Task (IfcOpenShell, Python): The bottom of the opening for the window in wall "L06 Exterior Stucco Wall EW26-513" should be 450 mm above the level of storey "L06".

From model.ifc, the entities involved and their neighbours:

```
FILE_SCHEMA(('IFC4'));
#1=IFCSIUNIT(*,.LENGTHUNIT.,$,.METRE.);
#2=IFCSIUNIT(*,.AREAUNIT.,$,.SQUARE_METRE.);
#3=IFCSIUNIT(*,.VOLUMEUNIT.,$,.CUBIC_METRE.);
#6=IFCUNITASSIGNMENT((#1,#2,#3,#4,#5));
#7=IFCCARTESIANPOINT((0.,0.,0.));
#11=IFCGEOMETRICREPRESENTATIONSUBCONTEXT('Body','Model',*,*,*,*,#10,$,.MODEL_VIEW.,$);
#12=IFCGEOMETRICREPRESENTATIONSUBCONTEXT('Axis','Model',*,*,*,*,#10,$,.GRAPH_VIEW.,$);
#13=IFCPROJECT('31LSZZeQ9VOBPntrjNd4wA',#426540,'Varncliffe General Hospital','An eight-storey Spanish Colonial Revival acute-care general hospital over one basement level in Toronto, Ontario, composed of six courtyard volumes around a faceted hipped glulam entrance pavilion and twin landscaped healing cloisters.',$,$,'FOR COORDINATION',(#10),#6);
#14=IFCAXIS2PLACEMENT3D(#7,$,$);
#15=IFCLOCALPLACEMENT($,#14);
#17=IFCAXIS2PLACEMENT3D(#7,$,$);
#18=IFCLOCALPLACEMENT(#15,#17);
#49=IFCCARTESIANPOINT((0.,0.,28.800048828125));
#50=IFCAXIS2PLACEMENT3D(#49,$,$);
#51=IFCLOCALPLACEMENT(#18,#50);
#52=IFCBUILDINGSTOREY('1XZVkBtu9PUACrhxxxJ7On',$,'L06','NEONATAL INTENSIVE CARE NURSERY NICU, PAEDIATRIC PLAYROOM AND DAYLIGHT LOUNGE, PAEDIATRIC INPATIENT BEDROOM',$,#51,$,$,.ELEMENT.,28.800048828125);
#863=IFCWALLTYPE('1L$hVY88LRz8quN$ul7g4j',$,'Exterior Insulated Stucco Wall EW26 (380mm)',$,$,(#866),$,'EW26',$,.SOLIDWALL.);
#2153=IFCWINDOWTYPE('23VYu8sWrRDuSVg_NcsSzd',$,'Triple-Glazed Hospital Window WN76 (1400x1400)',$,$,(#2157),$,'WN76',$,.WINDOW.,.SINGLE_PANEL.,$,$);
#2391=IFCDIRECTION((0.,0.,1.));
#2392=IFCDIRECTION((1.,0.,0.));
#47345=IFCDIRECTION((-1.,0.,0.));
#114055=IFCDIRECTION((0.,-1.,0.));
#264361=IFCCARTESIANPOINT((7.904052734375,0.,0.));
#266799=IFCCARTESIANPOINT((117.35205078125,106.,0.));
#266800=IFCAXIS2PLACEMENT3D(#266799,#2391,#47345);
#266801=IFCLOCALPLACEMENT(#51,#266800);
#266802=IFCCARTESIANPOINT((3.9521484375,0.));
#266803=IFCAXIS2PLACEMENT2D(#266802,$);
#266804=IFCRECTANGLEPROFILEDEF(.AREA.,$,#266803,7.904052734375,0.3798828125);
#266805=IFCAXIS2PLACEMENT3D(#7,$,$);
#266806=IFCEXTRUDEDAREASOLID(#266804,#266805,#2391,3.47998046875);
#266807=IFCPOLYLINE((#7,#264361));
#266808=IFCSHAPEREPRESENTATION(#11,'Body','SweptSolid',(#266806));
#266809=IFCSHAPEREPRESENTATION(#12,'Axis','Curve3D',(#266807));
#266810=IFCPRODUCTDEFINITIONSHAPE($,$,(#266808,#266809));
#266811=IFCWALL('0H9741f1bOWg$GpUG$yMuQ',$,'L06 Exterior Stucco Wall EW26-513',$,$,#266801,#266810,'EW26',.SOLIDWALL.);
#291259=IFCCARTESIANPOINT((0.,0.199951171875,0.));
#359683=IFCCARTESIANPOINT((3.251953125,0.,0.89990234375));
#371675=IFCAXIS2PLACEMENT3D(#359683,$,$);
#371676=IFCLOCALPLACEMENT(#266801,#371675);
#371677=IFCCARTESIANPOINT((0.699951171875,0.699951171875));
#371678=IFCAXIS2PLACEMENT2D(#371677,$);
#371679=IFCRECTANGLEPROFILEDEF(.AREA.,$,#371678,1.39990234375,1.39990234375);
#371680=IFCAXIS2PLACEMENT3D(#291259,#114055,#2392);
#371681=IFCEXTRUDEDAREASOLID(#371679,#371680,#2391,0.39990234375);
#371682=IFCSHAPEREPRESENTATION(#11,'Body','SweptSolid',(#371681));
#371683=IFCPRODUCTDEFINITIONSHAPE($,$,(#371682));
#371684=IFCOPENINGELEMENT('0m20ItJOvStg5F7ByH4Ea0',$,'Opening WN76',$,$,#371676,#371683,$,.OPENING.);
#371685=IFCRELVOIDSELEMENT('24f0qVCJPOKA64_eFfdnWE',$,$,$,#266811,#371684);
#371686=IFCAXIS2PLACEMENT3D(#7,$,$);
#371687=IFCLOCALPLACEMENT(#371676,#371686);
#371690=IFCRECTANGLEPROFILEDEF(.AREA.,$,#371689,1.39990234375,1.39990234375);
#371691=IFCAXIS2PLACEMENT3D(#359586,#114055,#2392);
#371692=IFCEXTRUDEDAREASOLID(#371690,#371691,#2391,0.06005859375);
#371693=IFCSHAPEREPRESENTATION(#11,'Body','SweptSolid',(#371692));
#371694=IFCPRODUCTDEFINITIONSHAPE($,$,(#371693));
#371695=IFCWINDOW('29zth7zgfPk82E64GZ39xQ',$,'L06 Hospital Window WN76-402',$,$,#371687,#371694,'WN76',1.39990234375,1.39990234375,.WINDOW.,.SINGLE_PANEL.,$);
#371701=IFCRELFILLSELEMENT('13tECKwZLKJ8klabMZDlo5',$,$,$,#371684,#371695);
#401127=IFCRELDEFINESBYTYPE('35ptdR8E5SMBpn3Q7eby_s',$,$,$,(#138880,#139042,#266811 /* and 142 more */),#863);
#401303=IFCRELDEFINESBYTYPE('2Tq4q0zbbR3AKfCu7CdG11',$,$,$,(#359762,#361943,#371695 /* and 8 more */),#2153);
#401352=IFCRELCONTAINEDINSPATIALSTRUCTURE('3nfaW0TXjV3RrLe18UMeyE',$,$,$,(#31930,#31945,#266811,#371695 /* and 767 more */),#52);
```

```python
import numpy as np
import ifcopenshell
import ifcopenshell.api.geometry
import ifcopenshell.geom
import ifcopenshell.util.element
import ifcopenshell.util.placement
import ifcopenshell.util.shape
import ifcopenshell.util.unit

model = ifcopenshell.open("model.ifc")
unit_scale = ifcopenshell.util.unit.calculate_unit_scale(model)

window = model.by_guid("29zth7zgfPk82E64GZ39xQ")
opening = window.FillsVoids[0].RelatingOpeningElement
storey = ifcopenshell.util.element.get_container(window, ifc_class="IfcBuildingStorey")
level = ifcopenshell.util.placement.get_local_placement(storey.ObjectPlacement)[2, 3]

# The opening's origin need not be at the sill, so measure its lowest point.
shape = ifcopenshell.geom.create_shape(ifcopenshell.geom.settings(), opening)
bottom = ifcopenshell.util.shape.get_shape_bottom_elevation(shape, shape.geometry) / unit_scale
dz = level + 0.45 / unit_scale - bottom

shift = np.array([0.0, 0.0, dz])
# The window is placed relative to its opening, so it follows when the opening moves.
matrix = ifcopenshell.util.placement.get_local_placement(opening.ObjectPlacement)
matrix[:3, 3] += shift
ifcopenshell.api.geometry.edit_object_placement(
    model, product=opening, matrix=matrix, is_si=False, should_transform_children=True
)

print(f"moved by {dz * unit_scale:+.3f} m")

model.write("model-out.ifc")
```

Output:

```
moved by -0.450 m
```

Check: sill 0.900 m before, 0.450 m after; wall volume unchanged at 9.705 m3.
